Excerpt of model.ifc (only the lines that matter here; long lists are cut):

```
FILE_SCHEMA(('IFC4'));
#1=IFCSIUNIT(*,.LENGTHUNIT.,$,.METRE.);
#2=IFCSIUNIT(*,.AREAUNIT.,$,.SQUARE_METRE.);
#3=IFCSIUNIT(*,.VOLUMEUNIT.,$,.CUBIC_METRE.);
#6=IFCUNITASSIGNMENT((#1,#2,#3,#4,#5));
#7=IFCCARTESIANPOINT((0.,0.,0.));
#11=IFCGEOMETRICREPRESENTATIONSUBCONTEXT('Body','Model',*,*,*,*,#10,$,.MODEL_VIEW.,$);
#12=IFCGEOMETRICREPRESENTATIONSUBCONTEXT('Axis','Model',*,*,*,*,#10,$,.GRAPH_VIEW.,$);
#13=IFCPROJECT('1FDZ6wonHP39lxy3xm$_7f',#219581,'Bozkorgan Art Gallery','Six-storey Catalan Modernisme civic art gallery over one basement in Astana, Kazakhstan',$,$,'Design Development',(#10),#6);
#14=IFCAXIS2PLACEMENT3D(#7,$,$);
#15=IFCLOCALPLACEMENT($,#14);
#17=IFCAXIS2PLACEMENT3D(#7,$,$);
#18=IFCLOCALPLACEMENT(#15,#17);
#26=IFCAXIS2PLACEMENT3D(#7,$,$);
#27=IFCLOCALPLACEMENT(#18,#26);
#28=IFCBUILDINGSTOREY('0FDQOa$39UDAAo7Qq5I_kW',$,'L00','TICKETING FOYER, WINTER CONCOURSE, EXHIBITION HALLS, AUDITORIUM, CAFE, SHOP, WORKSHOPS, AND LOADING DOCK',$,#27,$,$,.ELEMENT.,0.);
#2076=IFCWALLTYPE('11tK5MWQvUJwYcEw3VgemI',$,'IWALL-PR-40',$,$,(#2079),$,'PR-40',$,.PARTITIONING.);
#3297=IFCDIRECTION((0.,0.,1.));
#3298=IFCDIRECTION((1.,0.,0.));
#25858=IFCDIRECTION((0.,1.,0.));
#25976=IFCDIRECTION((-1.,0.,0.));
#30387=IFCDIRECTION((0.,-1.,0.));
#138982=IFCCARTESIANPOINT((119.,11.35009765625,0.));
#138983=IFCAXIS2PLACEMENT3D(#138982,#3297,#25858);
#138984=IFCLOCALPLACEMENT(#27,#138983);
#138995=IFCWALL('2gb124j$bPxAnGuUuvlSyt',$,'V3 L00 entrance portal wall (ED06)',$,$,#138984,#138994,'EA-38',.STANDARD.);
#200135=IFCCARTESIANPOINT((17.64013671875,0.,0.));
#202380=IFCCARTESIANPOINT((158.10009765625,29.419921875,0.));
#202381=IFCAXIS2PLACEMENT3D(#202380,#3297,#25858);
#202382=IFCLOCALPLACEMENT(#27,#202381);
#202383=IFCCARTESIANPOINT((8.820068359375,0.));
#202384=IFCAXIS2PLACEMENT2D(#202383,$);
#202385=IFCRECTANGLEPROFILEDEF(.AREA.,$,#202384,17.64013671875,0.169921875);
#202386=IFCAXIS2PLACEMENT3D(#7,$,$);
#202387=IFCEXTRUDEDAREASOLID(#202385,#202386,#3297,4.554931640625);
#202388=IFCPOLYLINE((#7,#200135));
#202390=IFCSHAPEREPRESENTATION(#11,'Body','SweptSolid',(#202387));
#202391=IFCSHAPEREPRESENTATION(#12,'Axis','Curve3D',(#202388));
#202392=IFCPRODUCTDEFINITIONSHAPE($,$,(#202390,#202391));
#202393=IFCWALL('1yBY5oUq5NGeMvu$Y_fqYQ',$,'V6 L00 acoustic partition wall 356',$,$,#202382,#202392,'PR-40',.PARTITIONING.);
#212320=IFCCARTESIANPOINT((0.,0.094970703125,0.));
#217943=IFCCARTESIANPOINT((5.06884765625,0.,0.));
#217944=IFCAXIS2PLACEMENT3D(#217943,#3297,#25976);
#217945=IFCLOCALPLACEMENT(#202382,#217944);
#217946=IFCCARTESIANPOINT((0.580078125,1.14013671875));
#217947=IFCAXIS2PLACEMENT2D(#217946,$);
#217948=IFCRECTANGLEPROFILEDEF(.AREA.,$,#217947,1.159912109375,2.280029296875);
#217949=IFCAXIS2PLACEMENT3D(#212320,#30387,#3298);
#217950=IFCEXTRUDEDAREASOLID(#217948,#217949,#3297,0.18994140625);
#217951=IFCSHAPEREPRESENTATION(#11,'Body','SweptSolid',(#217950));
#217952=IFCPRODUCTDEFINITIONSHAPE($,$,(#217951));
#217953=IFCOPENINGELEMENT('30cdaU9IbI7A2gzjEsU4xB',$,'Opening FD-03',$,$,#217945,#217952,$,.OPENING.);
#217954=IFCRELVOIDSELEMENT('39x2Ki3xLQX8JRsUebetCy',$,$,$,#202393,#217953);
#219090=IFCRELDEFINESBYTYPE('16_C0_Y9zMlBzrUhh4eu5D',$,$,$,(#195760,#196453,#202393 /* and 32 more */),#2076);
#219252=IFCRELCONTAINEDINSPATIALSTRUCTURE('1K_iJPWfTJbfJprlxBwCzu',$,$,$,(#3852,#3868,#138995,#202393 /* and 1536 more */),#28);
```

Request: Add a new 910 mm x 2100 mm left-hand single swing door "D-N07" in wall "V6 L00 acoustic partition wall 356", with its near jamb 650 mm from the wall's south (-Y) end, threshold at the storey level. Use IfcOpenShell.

```python
import numpy as np
import ifcopenshell
import ifcopenshell.api.feature
import ifcopenshell.api.geometry
import ifcopenshell.api.root
import ifcopenshell.api.spatial
import ifcopenshell.geom
import ifcopenshell.util.element
import ifcopenshell.util.placement
import ifcopenshell.util.representation
import ifcopenshell.util.shape
import ifcopenshell.util.unit

model = ifcopenshell.open("model.ifc")
unit_scale = ifcopenshell.util.unit.calculate_unit_scale(model)
settings = ifcopenshell.geom.settings()


def volume(element):
    """Net volume in cubic metres, openings subtracted."""
    shape = ifcopenshell.geom.create_shape(settings, element)
    return ifcopenshell.util.shape.get_volume(shape.geometry)


wall = model.by_guid("1yBY5oUq5NGeMvu$Y_fqYQ")
storey = ifcopenshell.util.element.get_container(wall, ifc_class="IfcBuildingStorey")
context = ifcopenshell.util.representation.get_context(model, "Model", "Body", "MODEL_VIEW")
before = volume(wall)

width, height, from_end, sill = 0.91, 2.1, 0.65, 0.0  # metres

# The wall runs along its own X axis, and the end named is its -X end.
wall_shape = ifcopenshell.geom.create_shape(settings, wall)
x, y, z = ifcopenshell.util.shape.get_vertices(wall_shape.geometry).T
start = x.min() + from_end
face, thickness = float(y.min()), float(y.max() - y.min())
wall_matrix = ifcopenshell.util.placement.get_local_placement(wall.ObjectPlacement)
level = ifcopenshell.util.placement.get_local_placement(storey.ObjectPlacement)[2, 3]


def in_wall(x, y):
    """Placement at x, y metres in the wall's axes, at sill height."""
    matrix = wall_matrix.copy()
    matrix[:, 3] = wall_matrix @ np.array([x / unit_scale, y / unit_scale, 0.0, 1.0])
    matrix[2, 3] = level + sill / unit_scale
    return matrix


# Opening: a box that overshoots both wall faces by 50 mm.
opening = ifcopenshell.api.root.create_entity(model, ifc_class="IfcOpeningElement", predefined_type="OPENING")
box = ifcopenshell.api.geometry.add_wall_representation(
    model, context=context, length=width, height=height, thickness=thickness + 0.1
)
ifcopenshell.api.geometry.assign_representation(model, product=opening, representation=box)
ifcopenshell.api.geometry.edit_object_placement(model, product=opening, matrix=in_wall(start, face - 0.05), is_si=False)
ifcopenshell.api.feature.add_feature(model, feature=opening, element=wall)

door = ifcopenshell.api.root.create_entity(model, ifc_class="IfcDoor", name="D-N07", predefined_type="DOOR")
door.OverallWidth, door.OverallHeight = width / unit_scale, height / unit_scale
door.OperationType = "SINGLE_SWING_LEFT"
body = ifcopenshell.api.geometry.add_door_representation(
    model,
    context=context,
    overall_width=door.OverallWidth,
    overall_height=door.OverallHeight,
    operation_type="SINGLE_SWING_LEFT",
    lining_properties={"LiningDepth": thickness / unit_scale, "ThresholdDepth": thickness / unit_scale},
)
ifcopenshell.api.geometry.assign_representation(model, product=door, representation=body)
ifcopenshell.api.spatial.assign_container(model, products=[door], relating_structure=storey)
ifcopenshell.api.feature.add_filling(model, opening=opening, element=door)

# The lining spans the wall, so the door starts at the wall face.
ifcopenshell.api.geometry.edit_object_placement(model, product=door, matrix=in_wall(start, face), is_si=False)

after = volume(wall)

print(f"wall volume {before:.3f} -> {after:.3f} m3")

model.write("model_updated.ifc")
```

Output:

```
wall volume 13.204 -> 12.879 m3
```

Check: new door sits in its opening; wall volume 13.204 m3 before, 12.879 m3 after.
